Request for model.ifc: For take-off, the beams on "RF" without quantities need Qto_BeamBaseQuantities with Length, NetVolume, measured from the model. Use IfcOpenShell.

First a look at what the model holds.

```python
import ifcopenshell
import ifcopenshell.util.element
import ifcopenshell.util.unit

model = ifcopenshell.open("model.ifc")
print(model.schema)
for unit_type in ("LENGTHUNIT", "AREAUNIT", "VOLUMEUNIT"):
    print(unit_type, ifcopenshell.util.unit.calculate_unit_scale(model, unit_type))
storey = next(s for s in model.by_type("IfcBuildingStorey") if s.Name == "RF")
beams = [e for e in ifcopenshell.util.element.get_decomposition(storey) if e.is_a("IfcBeam")]
for e in sorted(beams, key=lambda e: e.id()):
    print(e.id(), e.is_a(), e.Name, list(ifcopenshell.util.element.get_psets(e, qtos_only=True)), sep=" | ")
```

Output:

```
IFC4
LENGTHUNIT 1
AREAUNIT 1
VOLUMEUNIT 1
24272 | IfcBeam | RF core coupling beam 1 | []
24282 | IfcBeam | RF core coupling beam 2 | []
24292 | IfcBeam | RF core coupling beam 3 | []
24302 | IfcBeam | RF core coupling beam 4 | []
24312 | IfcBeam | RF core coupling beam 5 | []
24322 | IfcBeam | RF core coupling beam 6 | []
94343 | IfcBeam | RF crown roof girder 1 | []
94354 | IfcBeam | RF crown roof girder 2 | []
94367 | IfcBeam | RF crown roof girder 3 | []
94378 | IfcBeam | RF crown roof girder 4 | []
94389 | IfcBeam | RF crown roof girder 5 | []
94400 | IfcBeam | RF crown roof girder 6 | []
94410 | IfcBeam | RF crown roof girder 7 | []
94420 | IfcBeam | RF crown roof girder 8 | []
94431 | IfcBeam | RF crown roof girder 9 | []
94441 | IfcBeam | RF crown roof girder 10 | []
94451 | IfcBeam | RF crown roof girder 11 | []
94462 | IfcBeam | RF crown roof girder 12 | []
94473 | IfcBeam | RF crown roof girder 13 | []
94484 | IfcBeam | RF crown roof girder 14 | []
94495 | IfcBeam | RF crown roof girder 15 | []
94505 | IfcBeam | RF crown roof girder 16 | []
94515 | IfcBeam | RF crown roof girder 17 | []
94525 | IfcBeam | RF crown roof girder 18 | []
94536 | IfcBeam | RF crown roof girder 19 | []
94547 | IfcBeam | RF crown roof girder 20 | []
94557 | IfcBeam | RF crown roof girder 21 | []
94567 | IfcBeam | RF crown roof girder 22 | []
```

```python
import ifcopenshell
import ifcopenshell.api.pset
import ifcopenshell.geom
import ifcopenshell.util.element
import ifcopenshell.util.shape
import ifcopenshell.util.unit

model = ifcopenshell.open("model.ifc")
unit_scale = ifcopenshell.util.unit.calculate_unit_scale(model)
volume_scale = ifcopenshell.util.unit.calculate_unit_scale(model, "VOLUMEUNIT")
settings = ifcopenshell.geom.settings()

storey = next(s for s in model.by_type("IfcBuildingStorey") if s.Name == "RF")
beams = [e for e in ifcopenshell.util.element.get_decomposition(storey) if e.is_a("IfcBeam")]

for e in sorted(beams, key=lambda e: e.id()):
    if ifcopenshell.util.element.get_psets(e, qtos_only=True, should_inherit=False):
        continue
    # Geometry comes back in metres, in the element's own axes.
    shape = ifcopenshell.geom.create_shape(settings, e)
    values = {
        "Length": ifcopenshell.util.shape.get_max_xyz(shape.geometry) / unit_scale,
        "NetVolume": ifcopenshell.util.shape.get_volume(shape.geometry) / volume_scale,
    }
    qto = ifcopenshell.api.pset.add_qto(model, product=e, name="Qto_BeamBaseQuantities")
    ifcopenshell.api.pset.edit_qto(model, qto=qto, properties=values)
    print(e.id(), {k: round(v, 3) for k, v in values.items()})

model.write("model_edited.ifc")
```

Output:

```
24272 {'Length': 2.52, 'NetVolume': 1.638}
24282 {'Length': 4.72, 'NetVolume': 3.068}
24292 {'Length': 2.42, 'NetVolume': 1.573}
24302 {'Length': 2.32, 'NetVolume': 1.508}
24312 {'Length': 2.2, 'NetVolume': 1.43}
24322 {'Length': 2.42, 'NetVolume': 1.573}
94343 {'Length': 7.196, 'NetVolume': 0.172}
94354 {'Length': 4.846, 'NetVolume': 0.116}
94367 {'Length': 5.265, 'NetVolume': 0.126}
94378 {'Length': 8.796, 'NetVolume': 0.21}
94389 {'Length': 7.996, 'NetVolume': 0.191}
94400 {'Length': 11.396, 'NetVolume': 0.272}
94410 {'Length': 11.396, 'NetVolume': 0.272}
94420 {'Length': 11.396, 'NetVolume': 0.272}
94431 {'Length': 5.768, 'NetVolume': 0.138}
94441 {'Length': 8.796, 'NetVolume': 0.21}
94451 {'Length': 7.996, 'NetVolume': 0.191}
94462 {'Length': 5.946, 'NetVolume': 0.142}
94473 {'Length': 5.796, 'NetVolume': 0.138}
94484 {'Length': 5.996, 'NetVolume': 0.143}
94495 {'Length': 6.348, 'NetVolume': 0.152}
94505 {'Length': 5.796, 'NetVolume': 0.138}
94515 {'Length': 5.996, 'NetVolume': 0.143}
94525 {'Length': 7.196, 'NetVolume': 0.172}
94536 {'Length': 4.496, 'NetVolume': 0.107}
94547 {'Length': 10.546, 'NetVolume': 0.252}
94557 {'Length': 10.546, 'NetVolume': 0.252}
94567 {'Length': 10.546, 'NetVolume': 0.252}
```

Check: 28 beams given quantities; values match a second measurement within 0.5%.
